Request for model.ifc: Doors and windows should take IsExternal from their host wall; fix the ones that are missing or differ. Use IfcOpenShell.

First a look at what the model holds.

```python
import ifcopenshell
import ifcopenshell.util.element

model = ifcopenshell.open("model.ifc")
print(model.schema)
seen = {}
for e in model.by_type("IfcDoor") + model.by_type("IfcWindow"):
    if not e.FillsVoids:
        continue
    host = e.FillsVoids[0].RelatingOpeningElement.VoidsElements[0].RelatingBuildingElement
    own = ifcopenshell.util.element.get_pset(e, f"Pset_{e.is_a()[3:].removesuffix('StandardCase')}Common", "IsExternal")
    wall = ifcopenshell.util.element.get_pset(host, "Pset_WallCommon", "IsExternal")
    seen[e.is_a(), own, wall] = seen.get((e.is_a(), own, wall), 0) + 1
for (cls, own, wall), count in sorted(seen.items(), key=str):
    print(count, cls, "IsExternal:", own, "| host wall:", wall)
```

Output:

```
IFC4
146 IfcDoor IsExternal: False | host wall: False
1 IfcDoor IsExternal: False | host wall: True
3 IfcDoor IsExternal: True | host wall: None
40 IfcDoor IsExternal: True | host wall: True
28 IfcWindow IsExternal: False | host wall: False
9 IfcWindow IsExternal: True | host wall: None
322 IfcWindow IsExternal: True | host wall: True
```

```python
import ifcopenshell
import ifcopenshell.api.pset
import ifcopenshell.util.element

model = ifcopenshell.open("model.ifc")

count = 0
for ifc_class, pset_name in (("IfcDoor", "Pset_DoorCommon"), ("IfcWindow", "Pset_WindowCommon")):
    for e in model.by_type(ifc_class):
        if not e.FillsVoids:
            continue
        host = e.FillsVoids[0].RelatingOpeningElement.VoidsElements[0].RelatingBuildingElement
        external = ifcopenshell.util.element.get_pset(host, "Pset_WallCommon", "IsExternal")
        if external is None or ifcopenshell.util.element.get_pset(e, pset_name, "IsExternal") == external:
            continue
        pset = ifcopenshell.api.pset.add_pset(model, product=e, name=pset_name)
        ifcopenshell.api.pset.edit_pset(model, pset=pset, properties={"IsExternal": external})
        count += 1

print(count, "updated")

model.write("model_edited.ifc")
```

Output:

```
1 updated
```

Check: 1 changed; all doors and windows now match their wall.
